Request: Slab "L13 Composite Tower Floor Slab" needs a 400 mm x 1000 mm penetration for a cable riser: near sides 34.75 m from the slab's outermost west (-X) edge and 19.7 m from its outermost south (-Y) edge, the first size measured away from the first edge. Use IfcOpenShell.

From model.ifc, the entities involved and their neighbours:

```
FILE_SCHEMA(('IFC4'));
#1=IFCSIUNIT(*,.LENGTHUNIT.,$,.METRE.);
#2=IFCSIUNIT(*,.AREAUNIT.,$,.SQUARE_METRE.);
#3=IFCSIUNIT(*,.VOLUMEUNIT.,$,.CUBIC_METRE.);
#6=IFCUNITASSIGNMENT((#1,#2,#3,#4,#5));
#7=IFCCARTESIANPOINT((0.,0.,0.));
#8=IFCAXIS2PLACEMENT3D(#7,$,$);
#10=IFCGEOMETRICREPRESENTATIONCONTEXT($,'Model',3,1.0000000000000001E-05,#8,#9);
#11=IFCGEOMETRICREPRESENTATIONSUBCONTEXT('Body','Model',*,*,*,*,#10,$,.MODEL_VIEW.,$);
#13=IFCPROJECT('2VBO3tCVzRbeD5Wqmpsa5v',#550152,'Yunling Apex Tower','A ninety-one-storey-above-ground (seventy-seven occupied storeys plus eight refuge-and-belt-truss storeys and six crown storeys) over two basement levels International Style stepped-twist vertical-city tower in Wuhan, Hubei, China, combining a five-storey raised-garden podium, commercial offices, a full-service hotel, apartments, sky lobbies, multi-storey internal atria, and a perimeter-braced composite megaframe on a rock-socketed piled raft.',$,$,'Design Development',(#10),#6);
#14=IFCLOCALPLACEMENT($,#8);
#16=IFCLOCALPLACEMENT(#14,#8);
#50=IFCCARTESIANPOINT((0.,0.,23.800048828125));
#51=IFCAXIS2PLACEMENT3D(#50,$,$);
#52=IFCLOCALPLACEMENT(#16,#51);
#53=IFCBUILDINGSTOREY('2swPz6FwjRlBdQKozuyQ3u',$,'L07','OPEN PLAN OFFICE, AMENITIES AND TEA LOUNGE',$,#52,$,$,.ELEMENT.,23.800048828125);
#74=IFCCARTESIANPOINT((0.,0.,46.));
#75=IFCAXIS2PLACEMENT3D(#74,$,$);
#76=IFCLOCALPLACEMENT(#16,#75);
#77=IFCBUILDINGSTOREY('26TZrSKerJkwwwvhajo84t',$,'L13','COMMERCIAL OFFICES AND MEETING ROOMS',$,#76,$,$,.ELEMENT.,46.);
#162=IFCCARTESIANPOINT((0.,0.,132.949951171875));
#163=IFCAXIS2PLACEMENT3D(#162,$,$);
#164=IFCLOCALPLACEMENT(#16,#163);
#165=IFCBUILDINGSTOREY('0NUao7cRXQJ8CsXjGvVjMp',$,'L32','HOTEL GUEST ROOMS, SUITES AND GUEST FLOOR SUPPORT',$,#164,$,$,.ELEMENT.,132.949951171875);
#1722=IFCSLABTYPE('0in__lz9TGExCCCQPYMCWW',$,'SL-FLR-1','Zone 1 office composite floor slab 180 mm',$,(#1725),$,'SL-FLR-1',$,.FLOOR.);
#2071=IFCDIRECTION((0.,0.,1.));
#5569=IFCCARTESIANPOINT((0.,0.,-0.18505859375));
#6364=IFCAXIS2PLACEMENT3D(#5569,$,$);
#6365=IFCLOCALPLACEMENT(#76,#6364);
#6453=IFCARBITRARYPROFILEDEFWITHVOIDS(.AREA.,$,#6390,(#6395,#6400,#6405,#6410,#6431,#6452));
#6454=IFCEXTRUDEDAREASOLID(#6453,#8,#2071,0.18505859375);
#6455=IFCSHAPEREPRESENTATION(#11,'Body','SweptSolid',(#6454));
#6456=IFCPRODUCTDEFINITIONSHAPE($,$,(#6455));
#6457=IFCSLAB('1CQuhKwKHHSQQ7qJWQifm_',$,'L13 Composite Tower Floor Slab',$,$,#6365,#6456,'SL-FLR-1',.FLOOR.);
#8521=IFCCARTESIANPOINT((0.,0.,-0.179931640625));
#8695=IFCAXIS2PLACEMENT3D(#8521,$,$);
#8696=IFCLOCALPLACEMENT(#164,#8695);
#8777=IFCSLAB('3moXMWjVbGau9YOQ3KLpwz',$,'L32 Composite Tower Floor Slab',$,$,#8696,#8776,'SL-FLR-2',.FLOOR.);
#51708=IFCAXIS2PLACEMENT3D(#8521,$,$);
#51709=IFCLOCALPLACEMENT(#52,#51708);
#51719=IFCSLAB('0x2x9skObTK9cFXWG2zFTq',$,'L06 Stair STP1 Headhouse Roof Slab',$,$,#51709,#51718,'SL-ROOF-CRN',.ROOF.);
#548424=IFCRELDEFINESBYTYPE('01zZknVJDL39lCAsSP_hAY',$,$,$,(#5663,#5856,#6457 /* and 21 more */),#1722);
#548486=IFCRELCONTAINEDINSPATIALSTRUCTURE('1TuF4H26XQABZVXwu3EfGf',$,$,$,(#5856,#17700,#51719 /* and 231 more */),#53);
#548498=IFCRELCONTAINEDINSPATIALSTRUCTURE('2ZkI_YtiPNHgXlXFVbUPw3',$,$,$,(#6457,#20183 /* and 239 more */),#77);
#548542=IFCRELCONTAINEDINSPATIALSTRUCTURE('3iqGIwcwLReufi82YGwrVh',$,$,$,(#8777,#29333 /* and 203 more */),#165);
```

```python
import numpy as np
import ifcopenshell
import ifcopenshell.api.feature
import ifcopenshell.api.geometry
import ifcopenshell.api.root
import ifcopenshell.geom
import ifcopenshell.util.placement
import ifcopenshell.util.representation
import ifcopenshell.util.shape
import ifcopenshell.util.unit

model = ifcopenshell.open("model.ifc")
unit_scale = ifcopenshell.util.unit.calculate_unit_scale(model)
settings = ifcopenshell.geom.settings()


def volume(element):
    """Net volume in cubic metres, openings subtracted."""
    shape = ifcopenshell.geom.create_shape(settings, element)
    return ifcopenshell.util.shape.get_volume(shape.geometry)


slab = model.by_guid("1CQuhKwKHHSQQ7qJWQifm_")
before = volume(slab)

# Extent in the slab's own axes, in metres. The edges named are its -X and -Y sides.
slab_shape = ifcopenshell.geom.create_shape(settings, slab)
vertices = ifcopenshell.util.shape.get_vertices(slab_shape.geometry)
x_min, y_min, bottom = vertices.min(axis=0)
top = vertices[:, 2].max()

opening = ifcopenshell.api.root.create_entity(model, ifc_class="IfcOpeningElement", name="Cable riser opening", predefined_type="OPENING")
context = ifcopenshell.util.representation.get_context(model, "Model", "Body", "MODEL_VIEW")
width, depth = 0.4, 1
outline = [(0.0, 0.0), (width, 0.0), (width, depth), (0.0, depth), (0.0, 0.0)]
# Overshoot both faces by 50 mm so the cut is clean.
shape = ifcopenshell.api.geometry.add_slab_representation(
    model, context=context, depth=top - bottom + 0.1, polyline=outline
)
ifcopenshell.api.geometry.assign_representation(model, product=opening, representation=shape)

matrix = ifcopenshell.util.placement.get_local_placement(slab.ObjectPlacement)
matrix[:, 3] = matrix @ np.append(np.array([x_min + 34.75, y_min + 19.7, bottom - 0.05]) / unit_scale, 1.0)
ifcopenshell.api.geometry.edit_object_placement(model, product=opening, matrix=matrix, is_si=False)
ifcopenshell.api.feature.add_feature(model, feature=opening, element=slab)

after = volume(slab)

print(f"slab volume {before:.3f} -> {after:.3f} m3")

model.write("model_v2.ifc")
```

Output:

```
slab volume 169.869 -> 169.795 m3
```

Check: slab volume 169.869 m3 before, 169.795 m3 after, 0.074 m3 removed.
